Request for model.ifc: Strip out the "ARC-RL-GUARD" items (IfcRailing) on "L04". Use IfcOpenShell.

First a look at what the model holds.

```python
import ifcopenshell
import ifcopenshell.util.element

model = ifcopenshell.open("model.ifc")
print(model.schema)
storey = next(s for s in model.by_type("IfcBuildingStorey") if s.Name == "L04")
railings = [e for e in ifcopenshell.util.element.get_decomposition(storey) if e.is_a("IfcRailing")]
seen = {}
for e in railings:
    element_type = ifcopenshell.util.element.get_type(e)
    name = element_type.Name if element_type not in (None, e) else None
    seen[name] = seen.get(name, 0) + 1
for name, count in sorted(seen.items(), key=str):
    print(count, "x", name)
```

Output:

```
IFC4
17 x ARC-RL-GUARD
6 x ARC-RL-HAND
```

```python
import ifcopenshell
import ifcopenshell.api.root
import ifcopenshell.util.element

model = ifcopenshell.open("model.ifc")

storey = next(s for s in model.by_type("IfcBuildingStorey") if s.Name == "L04")
railings = [e for e in ifcopenshell.util.element.get_decomposition(storey) if e.is_a("IfcRailing")]
targets = [e for e in railings if (t := ifcopenshell.util.element.get_type(e)) not in (None, e) and t.Name == "ARC-RL-GUARD"]

for e in targets:
    ifcopenshell.api.root.remove_product(model, product=e)
print(len(targets), "removed")

model.write("model_edited.ifc")
```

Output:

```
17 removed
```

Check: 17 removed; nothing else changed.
